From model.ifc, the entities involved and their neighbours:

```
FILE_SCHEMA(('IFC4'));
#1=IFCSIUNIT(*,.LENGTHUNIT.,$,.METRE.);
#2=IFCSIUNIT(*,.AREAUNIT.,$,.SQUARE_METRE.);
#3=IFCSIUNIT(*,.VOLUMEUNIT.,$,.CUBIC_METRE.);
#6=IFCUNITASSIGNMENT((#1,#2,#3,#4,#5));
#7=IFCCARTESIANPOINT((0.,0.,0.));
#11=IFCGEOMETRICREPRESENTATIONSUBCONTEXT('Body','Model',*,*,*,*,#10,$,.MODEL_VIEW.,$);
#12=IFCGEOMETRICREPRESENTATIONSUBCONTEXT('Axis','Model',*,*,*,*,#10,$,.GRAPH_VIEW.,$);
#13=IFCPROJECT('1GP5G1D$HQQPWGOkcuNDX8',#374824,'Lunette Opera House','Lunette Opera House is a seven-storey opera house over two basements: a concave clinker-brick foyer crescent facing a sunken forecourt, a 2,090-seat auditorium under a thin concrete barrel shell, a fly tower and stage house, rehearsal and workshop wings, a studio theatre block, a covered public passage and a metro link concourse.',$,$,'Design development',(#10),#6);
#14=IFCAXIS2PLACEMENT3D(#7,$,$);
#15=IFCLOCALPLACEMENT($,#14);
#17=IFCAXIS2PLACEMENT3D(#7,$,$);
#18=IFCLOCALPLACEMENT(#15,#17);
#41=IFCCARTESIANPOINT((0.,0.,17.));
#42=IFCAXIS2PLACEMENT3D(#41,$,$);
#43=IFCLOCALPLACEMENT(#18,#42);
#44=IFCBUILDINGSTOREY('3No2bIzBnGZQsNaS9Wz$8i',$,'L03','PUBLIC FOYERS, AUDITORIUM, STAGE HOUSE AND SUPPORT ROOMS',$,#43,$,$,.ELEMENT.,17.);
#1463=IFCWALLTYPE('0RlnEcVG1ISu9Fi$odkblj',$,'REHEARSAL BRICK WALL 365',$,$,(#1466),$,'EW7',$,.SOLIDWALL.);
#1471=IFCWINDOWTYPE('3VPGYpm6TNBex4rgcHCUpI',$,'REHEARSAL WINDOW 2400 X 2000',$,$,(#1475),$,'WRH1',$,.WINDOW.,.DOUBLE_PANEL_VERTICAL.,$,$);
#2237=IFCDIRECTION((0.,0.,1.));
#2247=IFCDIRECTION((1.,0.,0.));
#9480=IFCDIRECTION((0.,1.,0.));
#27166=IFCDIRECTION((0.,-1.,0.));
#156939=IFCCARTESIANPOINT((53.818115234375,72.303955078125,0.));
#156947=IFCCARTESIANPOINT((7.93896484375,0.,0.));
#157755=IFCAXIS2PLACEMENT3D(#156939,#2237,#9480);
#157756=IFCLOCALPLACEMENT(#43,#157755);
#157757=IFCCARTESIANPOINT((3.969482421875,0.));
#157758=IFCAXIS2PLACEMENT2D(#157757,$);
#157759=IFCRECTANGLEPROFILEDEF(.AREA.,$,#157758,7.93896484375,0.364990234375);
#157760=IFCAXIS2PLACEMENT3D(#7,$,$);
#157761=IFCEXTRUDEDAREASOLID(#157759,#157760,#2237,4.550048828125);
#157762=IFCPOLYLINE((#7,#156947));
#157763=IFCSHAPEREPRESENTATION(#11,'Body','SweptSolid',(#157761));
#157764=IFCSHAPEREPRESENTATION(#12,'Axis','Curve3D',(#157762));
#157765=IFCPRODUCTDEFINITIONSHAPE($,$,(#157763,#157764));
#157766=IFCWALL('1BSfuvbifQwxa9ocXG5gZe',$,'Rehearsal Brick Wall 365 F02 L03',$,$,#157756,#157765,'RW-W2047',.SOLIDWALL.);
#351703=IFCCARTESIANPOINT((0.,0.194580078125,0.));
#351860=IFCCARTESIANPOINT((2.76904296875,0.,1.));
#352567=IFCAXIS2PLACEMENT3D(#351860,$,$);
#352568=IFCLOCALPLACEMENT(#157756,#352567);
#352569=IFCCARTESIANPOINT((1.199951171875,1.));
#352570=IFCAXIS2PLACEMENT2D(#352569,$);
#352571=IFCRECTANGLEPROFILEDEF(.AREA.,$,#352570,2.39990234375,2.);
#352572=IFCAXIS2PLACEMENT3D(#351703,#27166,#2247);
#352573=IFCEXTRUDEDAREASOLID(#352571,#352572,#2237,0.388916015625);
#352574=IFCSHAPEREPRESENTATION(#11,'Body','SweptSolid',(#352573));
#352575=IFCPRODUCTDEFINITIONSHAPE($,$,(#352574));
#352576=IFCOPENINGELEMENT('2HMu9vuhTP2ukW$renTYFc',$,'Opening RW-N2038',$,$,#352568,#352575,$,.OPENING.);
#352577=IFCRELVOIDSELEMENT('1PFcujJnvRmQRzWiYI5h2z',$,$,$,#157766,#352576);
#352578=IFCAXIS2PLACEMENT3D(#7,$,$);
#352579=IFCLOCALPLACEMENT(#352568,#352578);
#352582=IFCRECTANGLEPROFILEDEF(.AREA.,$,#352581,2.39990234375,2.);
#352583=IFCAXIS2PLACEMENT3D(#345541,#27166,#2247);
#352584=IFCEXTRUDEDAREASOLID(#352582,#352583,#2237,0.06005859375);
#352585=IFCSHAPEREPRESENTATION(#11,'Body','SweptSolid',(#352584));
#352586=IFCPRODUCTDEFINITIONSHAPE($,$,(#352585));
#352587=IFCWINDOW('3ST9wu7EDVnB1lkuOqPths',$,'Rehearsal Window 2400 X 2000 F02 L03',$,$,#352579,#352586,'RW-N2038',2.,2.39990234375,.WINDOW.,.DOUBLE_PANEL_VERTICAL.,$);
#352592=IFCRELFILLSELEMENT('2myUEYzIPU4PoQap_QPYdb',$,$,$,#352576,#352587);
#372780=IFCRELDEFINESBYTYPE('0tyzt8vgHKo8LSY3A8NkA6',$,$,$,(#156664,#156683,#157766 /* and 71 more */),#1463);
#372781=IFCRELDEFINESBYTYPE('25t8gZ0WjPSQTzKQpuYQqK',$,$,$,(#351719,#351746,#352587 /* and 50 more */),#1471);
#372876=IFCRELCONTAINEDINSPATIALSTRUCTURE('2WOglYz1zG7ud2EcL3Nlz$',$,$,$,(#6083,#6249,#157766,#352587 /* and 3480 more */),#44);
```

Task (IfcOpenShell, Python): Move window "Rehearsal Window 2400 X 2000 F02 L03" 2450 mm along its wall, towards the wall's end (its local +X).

```python
import ifcopenshell
import ifcopenshell.api.geometry
import ifcopenshell.util.placement
import ifcopenshell.util.unit

model = ifcopenshell.open("model.ifc")
unit_scale = ifcopenshell.util.unit.calculate_unit_scale(model)

window = model.by_guid("3ST9wu7EDVnB1lkuOqPths")
opening = window.FillsVoids[0].RelatingOpeningElement
wall = opening.VoidsElements[0].RelatingBuildingElement

wall_matrix = ifcopenshell.util.placement.get_local_placement(wall.ObjectPlacement)
shift = wall_matrix[:3, 0] * 2.45 / unit_scale
before = ifcopenshell.util.placement.get_local_placement(window.ObjectPlacement)[:3, 3].copy()

# The window is placed relative to its opening, so it follows when the opening moves.
matrix = ifcopenshell.util.placement.get_local_placement(opening.ObjectPlacement)
matrix[:3, 3] += shift
ifcopenshell.api.geometry.edit_object_placement(
    model, product=opening, matrix=matrix, is_si=False, should_transform_children=True
)

after = ifcopenshell.util.placement.get_local_placement(window.ObjectPlacement)[:3, 3]
print("window moved by", (after - before).round(3) + 0.0)

model.write("model_updated.ifc")
```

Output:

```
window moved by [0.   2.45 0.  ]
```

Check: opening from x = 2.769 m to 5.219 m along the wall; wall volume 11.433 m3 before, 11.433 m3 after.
